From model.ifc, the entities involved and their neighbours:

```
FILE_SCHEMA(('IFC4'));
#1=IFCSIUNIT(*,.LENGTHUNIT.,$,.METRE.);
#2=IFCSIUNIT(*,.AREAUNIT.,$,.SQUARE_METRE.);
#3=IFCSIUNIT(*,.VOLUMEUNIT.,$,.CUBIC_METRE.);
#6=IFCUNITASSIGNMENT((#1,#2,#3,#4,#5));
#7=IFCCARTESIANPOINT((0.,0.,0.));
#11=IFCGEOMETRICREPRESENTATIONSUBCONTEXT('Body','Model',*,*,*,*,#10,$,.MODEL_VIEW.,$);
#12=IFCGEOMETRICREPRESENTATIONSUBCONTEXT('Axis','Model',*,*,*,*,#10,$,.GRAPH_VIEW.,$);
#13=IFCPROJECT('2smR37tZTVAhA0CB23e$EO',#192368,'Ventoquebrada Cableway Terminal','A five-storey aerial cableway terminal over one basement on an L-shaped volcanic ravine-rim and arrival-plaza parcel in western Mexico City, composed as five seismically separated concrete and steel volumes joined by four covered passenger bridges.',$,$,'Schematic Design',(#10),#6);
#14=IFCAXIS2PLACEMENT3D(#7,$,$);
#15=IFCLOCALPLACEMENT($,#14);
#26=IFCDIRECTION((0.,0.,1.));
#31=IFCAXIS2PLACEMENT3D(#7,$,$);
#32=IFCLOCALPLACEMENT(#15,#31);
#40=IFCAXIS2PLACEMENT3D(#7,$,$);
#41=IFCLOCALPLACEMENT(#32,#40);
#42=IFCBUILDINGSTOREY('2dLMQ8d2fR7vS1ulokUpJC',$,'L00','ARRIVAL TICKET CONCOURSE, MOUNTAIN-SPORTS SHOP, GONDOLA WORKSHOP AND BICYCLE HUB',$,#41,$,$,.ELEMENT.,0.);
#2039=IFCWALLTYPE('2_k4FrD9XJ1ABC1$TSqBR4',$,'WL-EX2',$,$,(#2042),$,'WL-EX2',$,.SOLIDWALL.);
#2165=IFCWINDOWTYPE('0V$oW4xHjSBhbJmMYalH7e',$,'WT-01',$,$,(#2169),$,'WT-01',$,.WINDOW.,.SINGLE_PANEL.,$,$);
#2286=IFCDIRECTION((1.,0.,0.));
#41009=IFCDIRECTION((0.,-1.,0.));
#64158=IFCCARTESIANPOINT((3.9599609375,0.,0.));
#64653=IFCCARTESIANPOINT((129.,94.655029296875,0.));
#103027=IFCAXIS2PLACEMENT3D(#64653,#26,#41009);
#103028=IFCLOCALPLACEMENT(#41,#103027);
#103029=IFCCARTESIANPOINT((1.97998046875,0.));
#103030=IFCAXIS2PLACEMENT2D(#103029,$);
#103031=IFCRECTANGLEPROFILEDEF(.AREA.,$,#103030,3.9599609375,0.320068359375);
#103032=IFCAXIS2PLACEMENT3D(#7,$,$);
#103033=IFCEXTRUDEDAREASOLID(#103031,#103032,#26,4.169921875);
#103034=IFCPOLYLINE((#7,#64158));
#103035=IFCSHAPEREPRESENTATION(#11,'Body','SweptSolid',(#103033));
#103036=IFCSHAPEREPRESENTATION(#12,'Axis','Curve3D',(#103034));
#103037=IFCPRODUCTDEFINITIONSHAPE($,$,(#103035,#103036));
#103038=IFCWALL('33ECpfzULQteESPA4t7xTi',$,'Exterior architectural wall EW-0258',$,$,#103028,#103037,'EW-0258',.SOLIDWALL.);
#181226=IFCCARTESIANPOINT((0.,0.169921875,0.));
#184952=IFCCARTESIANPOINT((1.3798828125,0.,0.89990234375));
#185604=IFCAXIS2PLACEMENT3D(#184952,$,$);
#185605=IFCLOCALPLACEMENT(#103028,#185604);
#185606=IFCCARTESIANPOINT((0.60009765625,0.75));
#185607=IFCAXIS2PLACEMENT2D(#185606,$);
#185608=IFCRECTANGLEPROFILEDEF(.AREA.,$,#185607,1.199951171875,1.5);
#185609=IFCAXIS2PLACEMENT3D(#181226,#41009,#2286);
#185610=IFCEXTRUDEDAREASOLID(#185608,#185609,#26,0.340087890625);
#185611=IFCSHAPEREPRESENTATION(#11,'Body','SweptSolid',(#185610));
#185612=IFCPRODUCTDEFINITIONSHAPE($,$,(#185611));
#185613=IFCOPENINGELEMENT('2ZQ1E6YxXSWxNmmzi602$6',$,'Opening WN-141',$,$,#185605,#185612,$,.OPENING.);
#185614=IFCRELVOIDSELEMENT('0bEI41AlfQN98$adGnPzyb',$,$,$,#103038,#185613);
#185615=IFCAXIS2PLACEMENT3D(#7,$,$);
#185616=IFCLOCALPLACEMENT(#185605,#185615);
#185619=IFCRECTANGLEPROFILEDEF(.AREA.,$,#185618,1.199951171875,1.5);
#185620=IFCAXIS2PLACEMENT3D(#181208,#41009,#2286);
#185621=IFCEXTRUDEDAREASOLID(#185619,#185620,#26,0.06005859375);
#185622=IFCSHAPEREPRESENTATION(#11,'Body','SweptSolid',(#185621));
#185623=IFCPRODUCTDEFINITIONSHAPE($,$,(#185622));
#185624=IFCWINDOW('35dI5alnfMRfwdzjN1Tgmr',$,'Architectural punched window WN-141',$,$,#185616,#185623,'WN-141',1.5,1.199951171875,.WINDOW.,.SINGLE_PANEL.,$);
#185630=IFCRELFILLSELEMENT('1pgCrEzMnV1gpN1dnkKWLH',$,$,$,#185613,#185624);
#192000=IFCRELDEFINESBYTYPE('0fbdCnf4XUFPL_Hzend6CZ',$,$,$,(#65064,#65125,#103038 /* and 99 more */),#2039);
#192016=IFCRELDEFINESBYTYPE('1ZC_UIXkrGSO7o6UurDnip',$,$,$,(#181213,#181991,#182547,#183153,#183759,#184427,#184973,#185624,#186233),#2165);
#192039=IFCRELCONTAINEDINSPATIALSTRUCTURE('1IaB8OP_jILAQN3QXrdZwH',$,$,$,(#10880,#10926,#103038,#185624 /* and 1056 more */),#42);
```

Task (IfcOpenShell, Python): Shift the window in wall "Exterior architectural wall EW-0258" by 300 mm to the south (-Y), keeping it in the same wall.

```python
import ifcopenshell
import ifcopenshell.api.geometry
import ifcopenshell.util.placement

model = ifcopenshell.open("model.ifc")

window = model.by_guid("35dI5alnfMRfwdzjN1Tgmr")
opening = window.FillsVoids[0].RelatingOpeningElement
wall = opening.VoidsElements[0].RelatingBuildingElement

wall_matrix = ifcopenshell.util.placement.get_local_placement(wall.ObjectPlacement)
shift = wall_matrix[:3, 0] * 0.3
before = ifcopenshell.util.placement.get_local_placement(window.ObjectPlacement)[:3, 3].copy()

# The window is placed relative to its opening, so it follows when the opening moves.
matrix = ifcopenshell.util.placement.get_local_placement(opening.ObjectPlacement)
matrix[:3, 3] += shift
ifcopenshell.api.geometry.edit_object_placement(
    model, product=opening, matrix=matrix, is_si=False, should_transform_children=True
)

after = ifcopenshell.util.placement.get_local_placement(window.ObjectPlacement)[:3, 3]
print("window moved by", (after - before).round(3) + 0.0)

model.write("model_edited.ifc")
```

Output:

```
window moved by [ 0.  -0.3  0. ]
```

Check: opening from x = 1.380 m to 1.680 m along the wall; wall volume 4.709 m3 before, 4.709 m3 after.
